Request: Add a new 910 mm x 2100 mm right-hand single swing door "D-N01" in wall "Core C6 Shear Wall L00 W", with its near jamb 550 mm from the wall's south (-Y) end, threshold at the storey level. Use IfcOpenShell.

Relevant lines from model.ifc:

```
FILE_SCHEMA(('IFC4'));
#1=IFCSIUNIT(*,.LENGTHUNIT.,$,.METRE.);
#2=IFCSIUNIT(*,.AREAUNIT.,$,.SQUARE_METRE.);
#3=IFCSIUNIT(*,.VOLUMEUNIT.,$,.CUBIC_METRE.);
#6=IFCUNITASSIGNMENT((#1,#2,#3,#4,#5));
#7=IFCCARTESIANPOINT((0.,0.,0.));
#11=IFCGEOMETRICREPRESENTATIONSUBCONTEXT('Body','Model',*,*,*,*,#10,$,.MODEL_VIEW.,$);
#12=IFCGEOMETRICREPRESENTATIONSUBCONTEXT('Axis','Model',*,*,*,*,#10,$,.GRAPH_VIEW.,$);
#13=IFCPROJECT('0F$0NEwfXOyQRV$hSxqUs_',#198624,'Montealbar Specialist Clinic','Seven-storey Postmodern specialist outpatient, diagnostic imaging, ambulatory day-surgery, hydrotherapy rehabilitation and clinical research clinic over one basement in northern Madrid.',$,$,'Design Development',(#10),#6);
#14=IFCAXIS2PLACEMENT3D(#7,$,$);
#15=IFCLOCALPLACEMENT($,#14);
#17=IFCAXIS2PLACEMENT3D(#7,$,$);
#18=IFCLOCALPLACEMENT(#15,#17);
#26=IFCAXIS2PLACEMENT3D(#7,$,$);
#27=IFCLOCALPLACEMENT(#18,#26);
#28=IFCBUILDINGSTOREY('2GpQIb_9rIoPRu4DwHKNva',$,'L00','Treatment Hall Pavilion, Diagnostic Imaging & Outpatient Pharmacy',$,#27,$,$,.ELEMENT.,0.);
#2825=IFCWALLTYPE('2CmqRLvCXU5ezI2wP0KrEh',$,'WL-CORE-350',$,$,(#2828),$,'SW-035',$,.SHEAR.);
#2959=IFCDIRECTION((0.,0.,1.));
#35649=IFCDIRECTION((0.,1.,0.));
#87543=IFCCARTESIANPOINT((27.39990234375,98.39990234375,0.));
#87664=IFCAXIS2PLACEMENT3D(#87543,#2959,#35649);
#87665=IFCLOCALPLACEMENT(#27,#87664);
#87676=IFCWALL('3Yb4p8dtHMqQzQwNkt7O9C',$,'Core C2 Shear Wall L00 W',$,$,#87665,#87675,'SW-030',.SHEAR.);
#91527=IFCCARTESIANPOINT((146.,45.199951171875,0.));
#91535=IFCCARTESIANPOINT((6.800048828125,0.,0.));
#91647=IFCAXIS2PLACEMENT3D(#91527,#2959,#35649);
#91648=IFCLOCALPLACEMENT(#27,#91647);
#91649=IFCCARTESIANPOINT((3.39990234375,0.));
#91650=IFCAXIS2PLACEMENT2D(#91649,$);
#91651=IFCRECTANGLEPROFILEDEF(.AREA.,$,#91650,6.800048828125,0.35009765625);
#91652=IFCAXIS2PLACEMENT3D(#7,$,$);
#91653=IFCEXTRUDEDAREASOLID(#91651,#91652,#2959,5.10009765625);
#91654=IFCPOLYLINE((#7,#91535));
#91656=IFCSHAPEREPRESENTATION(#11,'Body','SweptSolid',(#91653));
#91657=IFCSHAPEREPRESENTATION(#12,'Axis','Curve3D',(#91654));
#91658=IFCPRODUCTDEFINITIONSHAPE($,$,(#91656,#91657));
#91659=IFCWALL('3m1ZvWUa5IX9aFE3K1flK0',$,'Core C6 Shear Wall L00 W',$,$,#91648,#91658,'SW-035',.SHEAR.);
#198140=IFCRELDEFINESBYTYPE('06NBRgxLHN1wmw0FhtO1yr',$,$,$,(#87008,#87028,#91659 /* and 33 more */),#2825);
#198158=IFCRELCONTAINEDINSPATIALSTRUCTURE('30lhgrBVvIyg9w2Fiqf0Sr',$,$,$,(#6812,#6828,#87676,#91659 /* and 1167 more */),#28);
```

```python
import numpy as np
import ifcopenshell
import ifcopenshell.api.feature
import ifcopenshell.api.geometry
import ifcopenshell.api.root
import ifcopenshell.api.spatial
import ifcopenshell.geom
import ifcopenshell.util.element
import ifcopenshell.util.placement
import ifcopenshell.util.representation
import ifcopenshell.util.shape
import ifcopenshell.util.unit

model = ifcopenshell.open("model.ifc")
unit_scale = ifcopenshell.util.unit.calculate_unit_scale(model)
settings = ifcopenshell.geom.settings()


def volume(element):
    """Net volume in cubic metres, openings subtracted."""
    shape = ifcopenshell.geom.create_shape(settings, element)
    return ifcopenshell.util.shape.get_volume(shape.geometry)


wall = model.by_id(91659)
storey = ifcopenshell.util.element.get_container(wall, ifc_class="IfcBuildingStorey")
context = ifcopenshell.util.representation.get_context(model, "Model", "Body", "MODEL_VIEW")
before = volume(wall)

width, height, from_end, sill = 0.91, 2.1, 0.55, 0.0  # metres

# The wall runs along its own X axis, and the end named is its -X end.
wall_shape = ifcopenshell.geom.create_shape(settings, wall)
x, y, z = ifcopenshell.util.shape.get_vertices(wall_shape.geometry).T
start = x.min() + from_end
face, thickness = float(y.min()), float(y.max() - y.min())
wall_matrix = ifcopenshell.util.placement.get_local_placement(wall.ObjectPlacement)
level = ifcopenshell.util.placement.get_local_placement(storey.ObjectPlacement)[2, 3]


def in_wall(x, y):
    """Placement at x, y metres in the wall's axes, at sill height."""
    matrix = wall_matrix.copy()
    matrix[:, 3] = wall_matrix @ np.array([x / unit_scale, y / unit_scale, 0.0, 1.0])
    matrix[2, 3] = level + sill / unit_scale
    return matrix


# Opening: a box that overshoots both wall faces by 50 mm.
opening = ifcopenshell.api.root.create_entity(model, ifc_class="IfcOpeningElement", predefined_type="OPENING")
box = ifcopenshell.api.geometry.add_wall_representation(
    model, context=context, length=width, height=height, thickness=thickness + 0.1
)
ifcopenshell.api.geometry.assign_representation(model, product=opening, representation=box)
ifcopenshell.api.geometry.edit_object_placement(model, product=opening, matrix=in_wall(start, face - 0.05), is_si=False)
ifcopenshell.api.feature.add_feature(model, feature=opening, element=wall)

door = ifcopenshell.api.root.create_entity(model, ifc_class="IfcDoor", name="D-N01", predefined_type="DOOR")
door.OverallWidth, door.OverallHeight = width / unit_scale, height / unit_scale
door.OperationType = "SINGLE_SWING_RIGHT"
body = ifcopenshell.api.geometry.add_door_representation(
    model,
    context=context,
    overall_width=door.OverallWidth,
    overall_height=door.OverallHeight,
    operation_type="SINGLE_SWING_RIGHT",
    lining_properties={"LiningDepth": thickness / unit_scale, "ThresholdDepth": thickness / unit_scale},
)
ifcopenshell.api.geometry.assign_representation(model, product=door, representation=body)
ifcopenshell.api.spatial.assign_container(model, products=[door], relating_structure=storey)
ifcopenshell.api.feature.add_filling(model, opening=opening, element=door)

# The lining spans the wall, so the door starts at the wall face.
ifcopenshell.api.geometry.edit_object_placement(model, product=door, matrix=in_wall(start, face), is_si=False)

after = volume(wall)

print(f"wall volume {before:.3f} -> {after:.3f} m3")

model.write("model_edited.ifc")
```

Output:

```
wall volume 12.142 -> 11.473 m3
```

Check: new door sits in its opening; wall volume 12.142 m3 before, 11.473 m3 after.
